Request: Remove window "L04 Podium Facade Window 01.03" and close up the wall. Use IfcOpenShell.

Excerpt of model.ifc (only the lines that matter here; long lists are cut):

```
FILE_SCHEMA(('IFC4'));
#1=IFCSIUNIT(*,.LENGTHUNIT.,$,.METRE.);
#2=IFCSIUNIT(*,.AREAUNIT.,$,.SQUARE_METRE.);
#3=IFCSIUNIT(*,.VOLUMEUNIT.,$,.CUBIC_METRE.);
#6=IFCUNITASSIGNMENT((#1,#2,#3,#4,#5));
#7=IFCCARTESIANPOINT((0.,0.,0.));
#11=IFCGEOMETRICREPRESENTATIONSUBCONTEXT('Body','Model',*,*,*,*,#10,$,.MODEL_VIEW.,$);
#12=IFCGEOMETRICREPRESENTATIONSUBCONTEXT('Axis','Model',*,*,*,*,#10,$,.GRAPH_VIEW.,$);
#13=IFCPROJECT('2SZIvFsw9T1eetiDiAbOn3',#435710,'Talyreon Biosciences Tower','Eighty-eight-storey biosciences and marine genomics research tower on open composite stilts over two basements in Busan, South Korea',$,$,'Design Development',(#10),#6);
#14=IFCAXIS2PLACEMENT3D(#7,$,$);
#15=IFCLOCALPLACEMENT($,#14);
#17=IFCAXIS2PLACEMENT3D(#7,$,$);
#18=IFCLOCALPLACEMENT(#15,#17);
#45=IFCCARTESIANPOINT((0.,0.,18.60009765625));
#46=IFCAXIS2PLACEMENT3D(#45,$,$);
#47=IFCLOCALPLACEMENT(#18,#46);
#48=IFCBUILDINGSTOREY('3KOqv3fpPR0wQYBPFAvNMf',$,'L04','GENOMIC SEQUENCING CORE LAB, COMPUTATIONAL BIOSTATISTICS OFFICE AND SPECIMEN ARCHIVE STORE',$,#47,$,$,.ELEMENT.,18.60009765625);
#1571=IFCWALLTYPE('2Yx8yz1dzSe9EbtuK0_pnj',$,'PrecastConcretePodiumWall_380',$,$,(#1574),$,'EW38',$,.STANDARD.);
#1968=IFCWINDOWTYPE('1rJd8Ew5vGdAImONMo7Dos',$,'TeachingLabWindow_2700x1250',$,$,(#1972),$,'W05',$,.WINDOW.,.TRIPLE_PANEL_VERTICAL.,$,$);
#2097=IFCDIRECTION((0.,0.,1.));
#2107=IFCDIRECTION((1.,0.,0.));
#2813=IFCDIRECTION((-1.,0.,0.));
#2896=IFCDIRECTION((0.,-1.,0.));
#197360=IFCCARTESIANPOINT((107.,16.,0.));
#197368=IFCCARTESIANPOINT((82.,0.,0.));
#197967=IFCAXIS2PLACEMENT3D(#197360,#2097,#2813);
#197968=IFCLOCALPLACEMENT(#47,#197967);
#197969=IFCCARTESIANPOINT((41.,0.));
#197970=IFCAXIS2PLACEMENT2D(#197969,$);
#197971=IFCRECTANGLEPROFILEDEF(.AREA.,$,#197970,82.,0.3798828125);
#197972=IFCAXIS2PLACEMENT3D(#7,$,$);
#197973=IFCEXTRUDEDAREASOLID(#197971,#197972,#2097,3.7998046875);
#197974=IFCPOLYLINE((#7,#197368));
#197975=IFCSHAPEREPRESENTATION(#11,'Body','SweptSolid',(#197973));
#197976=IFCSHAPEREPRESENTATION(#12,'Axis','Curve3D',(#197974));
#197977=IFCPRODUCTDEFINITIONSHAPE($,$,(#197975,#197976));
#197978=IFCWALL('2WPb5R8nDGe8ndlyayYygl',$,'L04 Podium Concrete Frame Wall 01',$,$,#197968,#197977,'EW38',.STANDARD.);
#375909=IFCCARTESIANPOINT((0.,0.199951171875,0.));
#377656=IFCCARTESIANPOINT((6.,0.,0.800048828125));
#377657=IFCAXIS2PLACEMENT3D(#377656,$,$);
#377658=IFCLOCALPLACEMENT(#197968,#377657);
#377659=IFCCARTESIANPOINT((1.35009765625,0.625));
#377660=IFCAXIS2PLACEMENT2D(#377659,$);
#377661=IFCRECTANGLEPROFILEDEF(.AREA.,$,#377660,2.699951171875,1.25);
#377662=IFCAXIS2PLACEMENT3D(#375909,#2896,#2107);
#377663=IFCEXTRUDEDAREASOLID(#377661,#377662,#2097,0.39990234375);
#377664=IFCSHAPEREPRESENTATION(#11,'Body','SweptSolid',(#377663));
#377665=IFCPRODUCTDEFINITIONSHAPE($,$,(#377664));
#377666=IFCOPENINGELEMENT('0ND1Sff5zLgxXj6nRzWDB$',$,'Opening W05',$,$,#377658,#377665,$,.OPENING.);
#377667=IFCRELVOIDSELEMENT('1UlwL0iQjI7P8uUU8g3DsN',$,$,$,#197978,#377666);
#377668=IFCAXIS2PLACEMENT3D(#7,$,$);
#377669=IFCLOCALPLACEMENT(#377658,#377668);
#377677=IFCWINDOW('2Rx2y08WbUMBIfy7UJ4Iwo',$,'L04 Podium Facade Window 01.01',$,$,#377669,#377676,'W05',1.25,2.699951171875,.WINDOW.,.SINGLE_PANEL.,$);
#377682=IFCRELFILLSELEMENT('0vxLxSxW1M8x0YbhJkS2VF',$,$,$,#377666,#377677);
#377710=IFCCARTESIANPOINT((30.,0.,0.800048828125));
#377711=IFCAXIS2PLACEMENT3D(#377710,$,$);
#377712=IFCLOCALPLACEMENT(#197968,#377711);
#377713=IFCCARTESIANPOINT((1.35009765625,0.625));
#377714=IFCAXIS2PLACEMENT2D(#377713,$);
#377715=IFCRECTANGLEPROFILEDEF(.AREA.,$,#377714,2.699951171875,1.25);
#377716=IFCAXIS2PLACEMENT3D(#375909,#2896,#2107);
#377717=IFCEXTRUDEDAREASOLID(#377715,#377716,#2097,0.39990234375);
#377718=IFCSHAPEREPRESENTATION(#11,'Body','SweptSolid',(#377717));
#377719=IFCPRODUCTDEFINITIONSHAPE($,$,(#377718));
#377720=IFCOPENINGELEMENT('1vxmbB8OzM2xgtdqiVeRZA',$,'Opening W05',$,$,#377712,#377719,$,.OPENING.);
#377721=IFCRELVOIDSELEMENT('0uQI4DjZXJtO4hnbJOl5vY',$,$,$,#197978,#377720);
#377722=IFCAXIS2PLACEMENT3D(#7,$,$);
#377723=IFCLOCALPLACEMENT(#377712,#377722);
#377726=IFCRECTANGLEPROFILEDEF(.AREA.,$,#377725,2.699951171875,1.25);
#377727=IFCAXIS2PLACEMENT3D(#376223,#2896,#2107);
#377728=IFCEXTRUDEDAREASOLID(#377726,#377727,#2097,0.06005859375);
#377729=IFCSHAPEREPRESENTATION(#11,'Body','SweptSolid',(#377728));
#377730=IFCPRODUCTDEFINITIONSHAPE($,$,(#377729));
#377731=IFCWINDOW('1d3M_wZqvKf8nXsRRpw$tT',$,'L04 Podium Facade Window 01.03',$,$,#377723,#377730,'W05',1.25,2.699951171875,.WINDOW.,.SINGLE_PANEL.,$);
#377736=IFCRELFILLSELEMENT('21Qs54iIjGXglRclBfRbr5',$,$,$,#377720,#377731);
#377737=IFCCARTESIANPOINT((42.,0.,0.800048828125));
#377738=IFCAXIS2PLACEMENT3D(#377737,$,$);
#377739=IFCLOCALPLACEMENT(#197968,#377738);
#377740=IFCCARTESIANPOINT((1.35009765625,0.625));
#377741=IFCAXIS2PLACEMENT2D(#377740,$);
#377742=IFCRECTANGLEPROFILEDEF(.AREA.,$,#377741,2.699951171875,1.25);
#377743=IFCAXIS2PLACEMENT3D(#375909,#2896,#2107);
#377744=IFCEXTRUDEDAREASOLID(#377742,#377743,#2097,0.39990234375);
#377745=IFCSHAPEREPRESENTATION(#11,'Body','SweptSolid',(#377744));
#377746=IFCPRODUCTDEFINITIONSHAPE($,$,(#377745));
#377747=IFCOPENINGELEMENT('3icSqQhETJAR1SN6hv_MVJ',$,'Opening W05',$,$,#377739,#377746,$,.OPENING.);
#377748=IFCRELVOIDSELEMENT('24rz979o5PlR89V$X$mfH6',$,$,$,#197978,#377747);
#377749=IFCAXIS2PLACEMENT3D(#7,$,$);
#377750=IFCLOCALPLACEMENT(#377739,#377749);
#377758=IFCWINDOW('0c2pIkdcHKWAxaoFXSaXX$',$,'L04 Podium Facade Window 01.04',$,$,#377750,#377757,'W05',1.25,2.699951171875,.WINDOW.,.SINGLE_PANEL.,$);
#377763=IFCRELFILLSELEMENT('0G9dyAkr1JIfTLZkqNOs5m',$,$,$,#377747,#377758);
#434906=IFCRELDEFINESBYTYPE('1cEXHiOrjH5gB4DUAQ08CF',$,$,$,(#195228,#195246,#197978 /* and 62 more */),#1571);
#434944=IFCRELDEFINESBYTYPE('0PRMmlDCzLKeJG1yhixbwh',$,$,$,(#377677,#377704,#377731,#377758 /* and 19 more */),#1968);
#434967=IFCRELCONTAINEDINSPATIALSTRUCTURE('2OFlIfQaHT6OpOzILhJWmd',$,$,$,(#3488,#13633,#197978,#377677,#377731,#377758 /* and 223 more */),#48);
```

```python
import ifcopenshell
import ifcopenshell.api.feature
import ifcopenshell.api.root
import ifcopenshell.geom
import ifcopenshell.util.shape

model = ifcopenshell.open("model.ifc")
settings = ifcopenshell.geom.settings()


def volume(element):
    """Net volume in cubic metres, openings subtracted."""
    shape = ifcopenshell.geom.create_shape(settings, element)
    return ifcopenshell.util.shape.get_volume(shape.geometry)


window = model.by_guid("1d3M_wZqvKf8nXsRRpw$tT")
opening = window.FillsVoids[0].RelatingOpeningElement
wall = opening.VoidsElements[0].RelatingBuildingElement
before = volume(wall)

ifcopenshell.api.root.remove_product(model, product=window)
ifcopenshell.api.feature.remove_feature(model, feature=opening)

after = volume(wall)

print(f"wall volume {before:.3f} -> {after:.3f} m3")

model.write("model_rev.ifc")
```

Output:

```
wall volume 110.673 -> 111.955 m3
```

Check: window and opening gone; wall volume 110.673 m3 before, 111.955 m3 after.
